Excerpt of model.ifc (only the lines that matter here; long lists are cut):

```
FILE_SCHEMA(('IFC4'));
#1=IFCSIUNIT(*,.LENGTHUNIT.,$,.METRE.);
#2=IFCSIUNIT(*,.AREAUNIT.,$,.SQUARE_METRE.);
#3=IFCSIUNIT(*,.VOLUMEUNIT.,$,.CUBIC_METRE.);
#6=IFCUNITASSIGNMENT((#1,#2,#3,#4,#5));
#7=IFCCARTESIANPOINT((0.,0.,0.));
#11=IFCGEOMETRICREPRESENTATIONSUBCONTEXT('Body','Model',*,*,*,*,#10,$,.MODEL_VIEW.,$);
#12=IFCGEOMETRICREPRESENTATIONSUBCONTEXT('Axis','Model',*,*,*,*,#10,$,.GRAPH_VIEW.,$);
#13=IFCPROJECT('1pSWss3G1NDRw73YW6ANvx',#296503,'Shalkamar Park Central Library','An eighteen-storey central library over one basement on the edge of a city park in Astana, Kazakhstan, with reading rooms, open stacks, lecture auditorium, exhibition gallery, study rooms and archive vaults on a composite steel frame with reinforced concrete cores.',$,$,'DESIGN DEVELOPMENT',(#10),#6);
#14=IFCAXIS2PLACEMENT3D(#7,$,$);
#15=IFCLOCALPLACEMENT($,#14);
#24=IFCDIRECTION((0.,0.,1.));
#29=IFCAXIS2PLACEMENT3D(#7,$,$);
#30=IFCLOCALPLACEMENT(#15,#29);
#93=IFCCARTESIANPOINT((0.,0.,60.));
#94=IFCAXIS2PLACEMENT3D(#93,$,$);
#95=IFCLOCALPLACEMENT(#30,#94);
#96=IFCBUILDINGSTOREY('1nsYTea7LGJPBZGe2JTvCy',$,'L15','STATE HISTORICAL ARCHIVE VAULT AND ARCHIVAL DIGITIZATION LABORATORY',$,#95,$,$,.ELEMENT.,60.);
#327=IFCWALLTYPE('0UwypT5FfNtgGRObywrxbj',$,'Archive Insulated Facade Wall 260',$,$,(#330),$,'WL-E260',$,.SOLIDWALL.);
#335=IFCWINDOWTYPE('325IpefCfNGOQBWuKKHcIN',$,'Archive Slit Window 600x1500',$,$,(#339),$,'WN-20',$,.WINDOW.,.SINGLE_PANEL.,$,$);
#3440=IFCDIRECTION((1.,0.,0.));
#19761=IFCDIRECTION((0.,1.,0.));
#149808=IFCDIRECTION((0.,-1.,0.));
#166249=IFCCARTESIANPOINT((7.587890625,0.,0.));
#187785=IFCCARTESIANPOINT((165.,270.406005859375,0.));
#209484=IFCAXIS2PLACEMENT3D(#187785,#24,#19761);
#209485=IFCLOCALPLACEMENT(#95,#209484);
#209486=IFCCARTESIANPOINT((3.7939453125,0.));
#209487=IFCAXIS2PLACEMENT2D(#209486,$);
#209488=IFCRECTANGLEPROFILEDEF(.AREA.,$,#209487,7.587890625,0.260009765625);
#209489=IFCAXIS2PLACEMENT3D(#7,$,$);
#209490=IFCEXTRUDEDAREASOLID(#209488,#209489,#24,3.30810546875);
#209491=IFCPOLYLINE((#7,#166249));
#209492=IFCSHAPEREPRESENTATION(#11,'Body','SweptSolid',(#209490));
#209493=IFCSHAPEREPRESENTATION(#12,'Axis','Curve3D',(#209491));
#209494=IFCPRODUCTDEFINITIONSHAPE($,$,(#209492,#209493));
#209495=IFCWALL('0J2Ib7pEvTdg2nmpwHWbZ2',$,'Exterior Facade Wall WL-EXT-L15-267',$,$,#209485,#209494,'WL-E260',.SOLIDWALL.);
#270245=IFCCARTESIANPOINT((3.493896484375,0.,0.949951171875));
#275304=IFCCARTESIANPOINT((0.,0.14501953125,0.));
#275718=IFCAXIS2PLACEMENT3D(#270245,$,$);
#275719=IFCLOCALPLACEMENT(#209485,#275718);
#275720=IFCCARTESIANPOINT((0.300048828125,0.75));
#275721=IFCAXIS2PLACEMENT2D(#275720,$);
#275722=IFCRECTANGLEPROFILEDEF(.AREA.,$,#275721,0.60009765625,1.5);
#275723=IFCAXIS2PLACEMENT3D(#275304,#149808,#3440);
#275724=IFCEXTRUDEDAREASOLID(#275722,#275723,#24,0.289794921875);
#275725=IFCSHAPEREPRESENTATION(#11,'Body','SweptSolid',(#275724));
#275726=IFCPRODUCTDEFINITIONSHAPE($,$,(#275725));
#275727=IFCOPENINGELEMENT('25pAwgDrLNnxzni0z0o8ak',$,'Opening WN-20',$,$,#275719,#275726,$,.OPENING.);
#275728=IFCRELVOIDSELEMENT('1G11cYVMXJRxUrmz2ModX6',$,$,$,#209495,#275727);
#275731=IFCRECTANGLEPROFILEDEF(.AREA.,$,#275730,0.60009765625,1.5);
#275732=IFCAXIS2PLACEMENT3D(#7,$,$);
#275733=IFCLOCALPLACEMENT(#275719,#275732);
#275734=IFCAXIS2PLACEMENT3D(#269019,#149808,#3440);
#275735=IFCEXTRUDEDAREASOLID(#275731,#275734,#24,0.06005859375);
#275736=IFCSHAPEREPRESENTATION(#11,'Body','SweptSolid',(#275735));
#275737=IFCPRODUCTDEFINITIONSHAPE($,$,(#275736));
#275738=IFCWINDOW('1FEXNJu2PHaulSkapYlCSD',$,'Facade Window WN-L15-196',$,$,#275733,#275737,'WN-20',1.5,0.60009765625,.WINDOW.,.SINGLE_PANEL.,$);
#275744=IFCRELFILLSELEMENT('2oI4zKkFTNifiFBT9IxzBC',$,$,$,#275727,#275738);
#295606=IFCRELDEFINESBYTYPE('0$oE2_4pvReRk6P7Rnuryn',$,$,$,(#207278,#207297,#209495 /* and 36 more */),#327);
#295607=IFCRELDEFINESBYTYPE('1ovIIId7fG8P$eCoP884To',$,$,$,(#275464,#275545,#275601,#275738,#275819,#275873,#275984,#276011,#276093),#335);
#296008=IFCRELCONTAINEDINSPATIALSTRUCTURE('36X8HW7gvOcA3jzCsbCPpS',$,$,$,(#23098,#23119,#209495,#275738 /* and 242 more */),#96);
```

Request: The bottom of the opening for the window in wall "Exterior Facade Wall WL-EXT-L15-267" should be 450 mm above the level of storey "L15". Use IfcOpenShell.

```python
import numpy as np
import ifcopenshell
import ifcopenshell.api.geometry
import ifcopenshell.geom
import ifcopenshell.util.element
import ifcopenshell.util.placement
import ifcopenshell.util.shape
import ifcopenshell.util.unit

model = ifcopenshell.open("model.ifc")
unit_scale = ifcopenshell.util.unit.calculate_unit_scale(model)

window = model.by_id(275738)
opening = window.FillsVoids[0].RelatingOpeningElement
storey = ifcopenshell.util.element.get_container(window, ifc_class="IfcBuildingStorey")
level = ifcopenshell.util.placement.get_local_placement(storey.ObjectPlacement)[2, 3]

# The opening's origin need not be at the sill, so measure its lowest point.
shape = ifcopenshell.geom.create_shape(ifcopenshell.geom.settings(), opening)
bottom = ifcopenshell.util.shape.get_shape_bottom_elevation(shape, shape.geometry) / unit_scale
dz = level + 0.45 - bottom

shift = np.array([0.0, 0.0, dz])
# The window is placed relative to its opening, so it follows when the opening moves.
matrix = ifcopenshell.util.placement.get_local_placement(opening.ObjectPlacement)
matrix[:3, 3] += shift
ifcopenshell.api.geometry.edit_object_placement(
    model, product=opening, matrix=matrix, is_si=False, should_transform_children=True
)

print(f"moved by {dz * unit_scale:+.3f} m")

model.write("model_edited.ifc")
```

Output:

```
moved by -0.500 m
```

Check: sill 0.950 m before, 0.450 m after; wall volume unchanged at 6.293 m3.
